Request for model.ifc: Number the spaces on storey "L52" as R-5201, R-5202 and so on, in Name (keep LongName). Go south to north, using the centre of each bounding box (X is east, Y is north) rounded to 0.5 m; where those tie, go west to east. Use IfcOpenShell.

First a look at what the model holds.

```python
import ifcopenshell
import ifcopenshell.util.element
import ifcopenshell.util.placement

model = ifcopenshell.open("model.ifc")
print(model.schema)
storey = next(s for s in model.by_type("IfcBuildingStorey") if s.Name == "L52")
spaces = [e for e in ifcopenshell.util.element.get_decomposition(storey) if e.is_a("IfcSpace")]
for e in sorted(spaces, key=lambda e: e.id()):
    origin = ifcopenshell.util.placement.get_local_placement(e.ObjectPlacement)[:3, 3]
    print(e.id(), e.Name, e.LongName, origin.round(2) + 0.0, sep=" | ")
```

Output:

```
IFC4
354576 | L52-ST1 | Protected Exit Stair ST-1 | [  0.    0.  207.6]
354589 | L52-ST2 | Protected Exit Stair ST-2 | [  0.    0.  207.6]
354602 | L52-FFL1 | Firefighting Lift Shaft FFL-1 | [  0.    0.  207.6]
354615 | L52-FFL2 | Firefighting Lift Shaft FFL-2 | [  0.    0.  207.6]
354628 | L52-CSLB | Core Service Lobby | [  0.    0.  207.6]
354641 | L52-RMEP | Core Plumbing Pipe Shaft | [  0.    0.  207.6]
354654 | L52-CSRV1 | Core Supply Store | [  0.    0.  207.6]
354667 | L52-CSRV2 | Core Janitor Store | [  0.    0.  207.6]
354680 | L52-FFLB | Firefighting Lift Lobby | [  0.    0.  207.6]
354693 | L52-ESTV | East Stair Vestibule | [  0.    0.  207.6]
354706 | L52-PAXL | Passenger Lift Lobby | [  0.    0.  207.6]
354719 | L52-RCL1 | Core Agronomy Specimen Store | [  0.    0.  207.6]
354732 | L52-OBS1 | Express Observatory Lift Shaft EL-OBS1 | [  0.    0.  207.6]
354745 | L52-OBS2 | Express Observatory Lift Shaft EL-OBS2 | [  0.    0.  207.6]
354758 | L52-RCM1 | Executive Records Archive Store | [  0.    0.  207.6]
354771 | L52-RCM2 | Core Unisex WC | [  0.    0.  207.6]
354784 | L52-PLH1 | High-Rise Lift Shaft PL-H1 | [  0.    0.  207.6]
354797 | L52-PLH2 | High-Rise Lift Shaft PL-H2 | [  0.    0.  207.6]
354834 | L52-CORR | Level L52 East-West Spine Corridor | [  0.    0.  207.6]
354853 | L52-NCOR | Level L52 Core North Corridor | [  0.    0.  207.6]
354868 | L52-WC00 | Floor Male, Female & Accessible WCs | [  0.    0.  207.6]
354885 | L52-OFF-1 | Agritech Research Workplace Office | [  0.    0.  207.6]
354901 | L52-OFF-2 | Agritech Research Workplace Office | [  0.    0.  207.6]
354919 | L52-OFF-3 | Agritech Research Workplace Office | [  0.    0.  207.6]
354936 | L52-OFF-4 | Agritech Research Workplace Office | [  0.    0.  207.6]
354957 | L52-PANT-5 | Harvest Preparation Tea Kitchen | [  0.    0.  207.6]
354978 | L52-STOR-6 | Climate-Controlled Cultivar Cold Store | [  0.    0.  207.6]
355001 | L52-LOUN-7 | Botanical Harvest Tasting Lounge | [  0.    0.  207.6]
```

```python
import ifcopenshell
import ifcopenshell.geom
import ifcopenshell.util.element
import ifcopenshell.util.shape

model = ifcopenshell.open("model.ifc")
settings = ifcopenshell.geom.settings()
settings.set("use-world-coords", True)


def centre(element):
    shape = ifcopenshell.geom.create_shape(settings, element)
    return ifcopenshell.util.shape.get_bbox_centroid(shape.geometry)


storey = next(s for s in model.by_type("IfcBuildingStorey") if s.Name == "L52")
spaces = [e for e in ifcopenshell.util.element.get_decomposition(storey) if e.is_a("IfcSpace")]

# Insertion points can sit at a corner or the storey origin, so sort by the geometry (in metres).
centres = {e: centre(e) for e in spaces}
spaces.sort(key=lambda e: (round(centres[e][1] / 0.5), centres[e][0]))

for i, e in enumerate(spaces, start=1):
    number = f"R-52{i:02d}"
    e.Name = number
    print(e.id(), number)

model.write("model-out.ifc")
```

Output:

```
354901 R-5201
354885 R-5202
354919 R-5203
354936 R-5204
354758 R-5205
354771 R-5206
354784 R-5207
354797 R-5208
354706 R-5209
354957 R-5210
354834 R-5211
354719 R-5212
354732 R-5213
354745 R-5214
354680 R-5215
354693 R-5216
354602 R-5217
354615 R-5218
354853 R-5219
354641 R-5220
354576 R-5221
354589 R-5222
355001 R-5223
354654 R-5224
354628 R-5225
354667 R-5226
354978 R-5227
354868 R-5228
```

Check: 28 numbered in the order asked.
